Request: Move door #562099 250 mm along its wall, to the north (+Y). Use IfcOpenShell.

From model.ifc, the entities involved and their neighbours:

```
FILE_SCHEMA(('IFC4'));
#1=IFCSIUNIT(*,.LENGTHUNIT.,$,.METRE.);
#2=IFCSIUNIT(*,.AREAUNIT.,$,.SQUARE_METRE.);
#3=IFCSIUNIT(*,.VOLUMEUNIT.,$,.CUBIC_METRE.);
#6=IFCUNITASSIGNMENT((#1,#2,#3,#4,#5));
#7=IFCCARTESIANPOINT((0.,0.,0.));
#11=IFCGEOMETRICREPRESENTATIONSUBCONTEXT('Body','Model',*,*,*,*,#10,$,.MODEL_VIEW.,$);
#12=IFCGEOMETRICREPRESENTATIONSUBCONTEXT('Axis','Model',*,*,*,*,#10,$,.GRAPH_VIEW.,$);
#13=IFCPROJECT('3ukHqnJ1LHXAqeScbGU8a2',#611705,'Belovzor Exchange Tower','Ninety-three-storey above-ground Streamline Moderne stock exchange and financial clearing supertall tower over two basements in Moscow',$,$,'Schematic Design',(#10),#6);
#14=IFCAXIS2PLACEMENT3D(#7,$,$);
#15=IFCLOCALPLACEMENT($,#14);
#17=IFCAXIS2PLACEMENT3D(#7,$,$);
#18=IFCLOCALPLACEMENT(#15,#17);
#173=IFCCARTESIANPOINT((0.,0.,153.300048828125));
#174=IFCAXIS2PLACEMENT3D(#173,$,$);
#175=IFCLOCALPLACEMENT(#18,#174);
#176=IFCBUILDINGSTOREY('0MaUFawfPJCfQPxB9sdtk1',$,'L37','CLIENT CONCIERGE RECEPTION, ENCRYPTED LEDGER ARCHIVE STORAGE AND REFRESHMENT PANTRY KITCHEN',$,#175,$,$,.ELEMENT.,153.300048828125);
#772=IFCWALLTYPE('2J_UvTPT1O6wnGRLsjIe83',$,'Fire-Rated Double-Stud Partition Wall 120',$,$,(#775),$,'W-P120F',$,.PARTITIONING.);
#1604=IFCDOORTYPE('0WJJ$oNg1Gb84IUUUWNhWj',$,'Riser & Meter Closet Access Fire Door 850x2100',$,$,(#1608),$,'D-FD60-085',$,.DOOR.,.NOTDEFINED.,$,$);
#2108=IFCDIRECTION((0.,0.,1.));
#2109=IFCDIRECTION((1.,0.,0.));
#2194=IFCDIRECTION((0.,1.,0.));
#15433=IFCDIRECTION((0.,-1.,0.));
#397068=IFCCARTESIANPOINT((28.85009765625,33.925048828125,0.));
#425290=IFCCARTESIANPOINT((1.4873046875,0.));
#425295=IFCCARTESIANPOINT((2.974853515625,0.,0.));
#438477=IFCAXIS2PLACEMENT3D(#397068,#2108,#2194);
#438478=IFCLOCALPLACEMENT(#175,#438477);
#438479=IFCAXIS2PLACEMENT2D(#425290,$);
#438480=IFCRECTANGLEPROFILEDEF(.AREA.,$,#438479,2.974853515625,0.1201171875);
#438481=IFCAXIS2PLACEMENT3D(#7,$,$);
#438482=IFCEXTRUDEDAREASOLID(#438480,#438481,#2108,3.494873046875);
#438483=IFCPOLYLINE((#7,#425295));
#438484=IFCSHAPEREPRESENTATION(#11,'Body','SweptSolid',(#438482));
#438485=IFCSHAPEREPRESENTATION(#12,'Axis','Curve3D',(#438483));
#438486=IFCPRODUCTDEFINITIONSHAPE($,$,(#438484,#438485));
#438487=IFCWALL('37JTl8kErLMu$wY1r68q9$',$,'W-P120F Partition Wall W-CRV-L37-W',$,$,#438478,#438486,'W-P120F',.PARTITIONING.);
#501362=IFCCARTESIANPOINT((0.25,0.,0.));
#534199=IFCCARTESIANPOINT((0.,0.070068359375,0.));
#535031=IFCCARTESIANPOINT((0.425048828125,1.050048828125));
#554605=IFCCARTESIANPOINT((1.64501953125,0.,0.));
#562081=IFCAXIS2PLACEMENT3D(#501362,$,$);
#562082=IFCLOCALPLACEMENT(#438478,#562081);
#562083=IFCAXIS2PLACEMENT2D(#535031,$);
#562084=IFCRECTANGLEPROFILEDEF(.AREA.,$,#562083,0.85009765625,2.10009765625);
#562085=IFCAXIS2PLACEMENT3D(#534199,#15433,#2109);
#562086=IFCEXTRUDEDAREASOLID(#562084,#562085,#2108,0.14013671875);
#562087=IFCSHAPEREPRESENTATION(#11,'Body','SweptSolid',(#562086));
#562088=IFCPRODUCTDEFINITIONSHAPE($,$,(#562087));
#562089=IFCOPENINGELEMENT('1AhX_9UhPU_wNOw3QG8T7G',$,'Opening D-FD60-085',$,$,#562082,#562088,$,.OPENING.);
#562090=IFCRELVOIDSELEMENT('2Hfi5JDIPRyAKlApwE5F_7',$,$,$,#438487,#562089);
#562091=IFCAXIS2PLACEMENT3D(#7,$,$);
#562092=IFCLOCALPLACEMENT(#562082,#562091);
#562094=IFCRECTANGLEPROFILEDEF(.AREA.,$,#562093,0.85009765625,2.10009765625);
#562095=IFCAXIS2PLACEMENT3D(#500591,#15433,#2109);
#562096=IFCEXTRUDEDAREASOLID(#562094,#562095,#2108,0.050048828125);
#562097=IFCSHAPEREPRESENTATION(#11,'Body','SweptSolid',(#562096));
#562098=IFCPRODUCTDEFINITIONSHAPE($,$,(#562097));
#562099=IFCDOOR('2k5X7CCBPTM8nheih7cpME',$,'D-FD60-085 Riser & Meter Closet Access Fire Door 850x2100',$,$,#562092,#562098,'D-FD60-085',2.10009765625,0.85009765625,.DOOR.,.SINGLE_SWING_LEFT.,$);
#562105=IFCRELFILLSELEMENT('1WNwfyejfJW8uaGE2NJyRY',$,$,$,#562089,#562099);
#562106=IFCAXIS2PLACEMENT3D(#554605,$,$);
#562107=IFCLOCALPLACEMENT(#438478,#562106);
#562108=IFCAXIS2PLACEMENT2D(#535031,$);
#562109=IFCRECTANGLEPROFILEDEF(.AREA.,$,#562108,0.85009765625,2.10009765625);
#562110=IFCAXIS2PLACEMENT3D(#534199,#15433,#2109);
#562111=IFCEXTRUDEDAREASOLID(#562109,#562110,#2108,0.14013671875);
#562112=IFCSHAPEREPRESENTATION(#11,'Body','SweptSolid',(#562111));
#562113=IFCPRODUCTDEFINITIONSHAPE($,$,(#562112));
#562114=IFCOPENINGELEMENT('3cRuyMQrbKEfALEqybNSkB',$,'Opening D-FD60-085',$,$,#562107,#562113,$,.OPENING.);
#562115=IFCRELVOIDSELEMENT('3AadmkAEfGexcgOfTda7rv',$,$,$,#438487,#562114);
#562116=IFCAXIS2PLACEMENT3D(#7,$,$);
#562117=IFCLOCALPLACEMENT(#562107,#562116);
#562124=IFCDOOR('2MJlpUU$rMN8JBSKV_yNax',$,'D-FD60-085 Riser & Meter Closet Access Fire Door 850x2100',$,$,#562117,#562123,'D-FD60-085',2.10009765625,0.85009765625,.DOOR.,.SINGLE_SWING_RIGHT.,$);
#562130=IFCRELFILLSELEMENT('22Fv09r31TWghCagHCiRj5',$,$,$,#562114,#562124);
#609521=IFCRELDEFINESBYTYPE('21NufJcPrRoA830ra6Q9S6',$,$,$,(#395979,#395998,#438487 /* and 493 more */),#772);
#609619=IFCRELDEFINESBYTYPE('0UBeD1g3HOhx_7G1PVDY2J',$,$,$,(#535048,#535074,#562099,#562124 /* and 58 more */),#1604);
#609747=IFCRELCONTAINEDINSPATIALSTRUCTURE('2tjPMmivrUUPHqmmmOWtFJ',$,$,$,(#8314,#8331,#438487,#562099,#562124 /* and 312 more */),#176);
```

```python
import ifcopenshell
import ifcopenshell.api.geometry
import ifcopenshell.util.placement

model = ifcopenshell.open("model.ifc")

door = model.by_guid("2k5X7CCBPTM8nheih7cpME")
opening = door.FillsVoids[0].RelatingOpeningElement
wall = opening.VoidsElements[0].RelatingBuildingElement

wall_matrix = ifcopenshell.util.placement.get_local_placement(wall.ObjectPlacement)
shift = wall_matrix[:3, 0] * 0.25
before = ifcopenshell.util.placement.get_local_placement(door.ObjectPlacement)[:3, 3].copy()

# The door is placed relative to its opening, so it follows when the opening moves.
matrix = ifcopenshell.util.placement.get_local_placement(opening.ObjectPlacement)
matrix[:3, 3] += shift
ifcopenshell.api.geometry.edit_object_placement(
    model, product=opening, matrix=matrix, is_si=False, should_transform_children=True
)

after = ifcopenshell.util.placement.get_local_placement(door.ObjectPlacement)[:3, 3]
print("door moved by", (after - before).round(3) + 0.0)

model.write("model-out.ifc")
```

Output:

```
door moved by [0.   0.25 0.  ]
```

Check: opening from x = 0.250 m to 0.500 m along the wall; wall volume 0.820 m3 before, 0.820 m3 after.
